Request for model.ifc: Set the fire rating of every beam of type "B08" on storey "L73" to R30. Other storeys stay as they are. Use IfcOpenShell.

First a look at what the model holds.

```python
import ifcopenshell
import ifcopenshell.util.element

model = ifcopenshell.open("model.ifc")
print(model.schema)
storey = next(s for s in model.by_type("IfcBuildingStorey") if s.Name == "L73")
beams = [e for e in ifcopenshell.util.element.get_decomposition(storey) if e.is_a("IfcBeam")]
seen = {}
for e in beams:
    element_type = ifcopenshell.util.element.get_type(e)
    key = (element_type.Name if element_type != e and element_type else None, ifcopenshell.util.element.get_pset(e, "Pset_BeamCommon", "FireRating"))
    seen[key] = seen.get(key, 0) + 1
for (name, value), count in sorted(seen.items(), key=str):
    print(count, "x", name, "|", value)
```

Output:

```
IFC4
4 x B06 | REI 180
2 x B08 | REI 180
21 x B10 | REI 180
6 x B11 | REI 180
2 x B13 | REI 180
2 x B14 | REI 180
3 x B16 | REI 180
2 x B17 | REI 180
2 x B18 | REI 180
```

```python
import ifcopenshell
import ifcopenshell.api.pset
import ifcopenshell.util.element

model = ifcopenshell.open("model.ifc")

storey = next(s for s in model.by_type("IfcBuildingStorey") if s.Name == "L73")
beams = [e for e in ifcopenshell.util.element.get_decomposition(storey) if e.is_a("IfcBeam")]

count = 0
for e in beams:
    element_type = ifcopenshell.util.element.get_type(e)
    if element_type in (None, e) or element_type.Name != "B08":
        continue
    found = ifcopenshell.util.element.get_pset(e, "Pset_BeamCommon", should_inherit=False)
    if found:
        pset = model.by_id(found["id"])
        if len(ifcopenshell.util.element.get_elements_by_pset(pset)) > 1:
            pset = ifcopenshell.api.pset.unshare_pset(model, products=[e], pset=pset)[0]
    else:
        pset = ifcopenshell.api.pset.add_pset(model, product=e, name="Pset_BeamCommon")
    ifcopenshell.api.pset.edit_pset(model, pset=pset, properties={"FireRating": "R30"})
    count += 1

print(count, "beams updated")

model.write("model_edited.ifc")
```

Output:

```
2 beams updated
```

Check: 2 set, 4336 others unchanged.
